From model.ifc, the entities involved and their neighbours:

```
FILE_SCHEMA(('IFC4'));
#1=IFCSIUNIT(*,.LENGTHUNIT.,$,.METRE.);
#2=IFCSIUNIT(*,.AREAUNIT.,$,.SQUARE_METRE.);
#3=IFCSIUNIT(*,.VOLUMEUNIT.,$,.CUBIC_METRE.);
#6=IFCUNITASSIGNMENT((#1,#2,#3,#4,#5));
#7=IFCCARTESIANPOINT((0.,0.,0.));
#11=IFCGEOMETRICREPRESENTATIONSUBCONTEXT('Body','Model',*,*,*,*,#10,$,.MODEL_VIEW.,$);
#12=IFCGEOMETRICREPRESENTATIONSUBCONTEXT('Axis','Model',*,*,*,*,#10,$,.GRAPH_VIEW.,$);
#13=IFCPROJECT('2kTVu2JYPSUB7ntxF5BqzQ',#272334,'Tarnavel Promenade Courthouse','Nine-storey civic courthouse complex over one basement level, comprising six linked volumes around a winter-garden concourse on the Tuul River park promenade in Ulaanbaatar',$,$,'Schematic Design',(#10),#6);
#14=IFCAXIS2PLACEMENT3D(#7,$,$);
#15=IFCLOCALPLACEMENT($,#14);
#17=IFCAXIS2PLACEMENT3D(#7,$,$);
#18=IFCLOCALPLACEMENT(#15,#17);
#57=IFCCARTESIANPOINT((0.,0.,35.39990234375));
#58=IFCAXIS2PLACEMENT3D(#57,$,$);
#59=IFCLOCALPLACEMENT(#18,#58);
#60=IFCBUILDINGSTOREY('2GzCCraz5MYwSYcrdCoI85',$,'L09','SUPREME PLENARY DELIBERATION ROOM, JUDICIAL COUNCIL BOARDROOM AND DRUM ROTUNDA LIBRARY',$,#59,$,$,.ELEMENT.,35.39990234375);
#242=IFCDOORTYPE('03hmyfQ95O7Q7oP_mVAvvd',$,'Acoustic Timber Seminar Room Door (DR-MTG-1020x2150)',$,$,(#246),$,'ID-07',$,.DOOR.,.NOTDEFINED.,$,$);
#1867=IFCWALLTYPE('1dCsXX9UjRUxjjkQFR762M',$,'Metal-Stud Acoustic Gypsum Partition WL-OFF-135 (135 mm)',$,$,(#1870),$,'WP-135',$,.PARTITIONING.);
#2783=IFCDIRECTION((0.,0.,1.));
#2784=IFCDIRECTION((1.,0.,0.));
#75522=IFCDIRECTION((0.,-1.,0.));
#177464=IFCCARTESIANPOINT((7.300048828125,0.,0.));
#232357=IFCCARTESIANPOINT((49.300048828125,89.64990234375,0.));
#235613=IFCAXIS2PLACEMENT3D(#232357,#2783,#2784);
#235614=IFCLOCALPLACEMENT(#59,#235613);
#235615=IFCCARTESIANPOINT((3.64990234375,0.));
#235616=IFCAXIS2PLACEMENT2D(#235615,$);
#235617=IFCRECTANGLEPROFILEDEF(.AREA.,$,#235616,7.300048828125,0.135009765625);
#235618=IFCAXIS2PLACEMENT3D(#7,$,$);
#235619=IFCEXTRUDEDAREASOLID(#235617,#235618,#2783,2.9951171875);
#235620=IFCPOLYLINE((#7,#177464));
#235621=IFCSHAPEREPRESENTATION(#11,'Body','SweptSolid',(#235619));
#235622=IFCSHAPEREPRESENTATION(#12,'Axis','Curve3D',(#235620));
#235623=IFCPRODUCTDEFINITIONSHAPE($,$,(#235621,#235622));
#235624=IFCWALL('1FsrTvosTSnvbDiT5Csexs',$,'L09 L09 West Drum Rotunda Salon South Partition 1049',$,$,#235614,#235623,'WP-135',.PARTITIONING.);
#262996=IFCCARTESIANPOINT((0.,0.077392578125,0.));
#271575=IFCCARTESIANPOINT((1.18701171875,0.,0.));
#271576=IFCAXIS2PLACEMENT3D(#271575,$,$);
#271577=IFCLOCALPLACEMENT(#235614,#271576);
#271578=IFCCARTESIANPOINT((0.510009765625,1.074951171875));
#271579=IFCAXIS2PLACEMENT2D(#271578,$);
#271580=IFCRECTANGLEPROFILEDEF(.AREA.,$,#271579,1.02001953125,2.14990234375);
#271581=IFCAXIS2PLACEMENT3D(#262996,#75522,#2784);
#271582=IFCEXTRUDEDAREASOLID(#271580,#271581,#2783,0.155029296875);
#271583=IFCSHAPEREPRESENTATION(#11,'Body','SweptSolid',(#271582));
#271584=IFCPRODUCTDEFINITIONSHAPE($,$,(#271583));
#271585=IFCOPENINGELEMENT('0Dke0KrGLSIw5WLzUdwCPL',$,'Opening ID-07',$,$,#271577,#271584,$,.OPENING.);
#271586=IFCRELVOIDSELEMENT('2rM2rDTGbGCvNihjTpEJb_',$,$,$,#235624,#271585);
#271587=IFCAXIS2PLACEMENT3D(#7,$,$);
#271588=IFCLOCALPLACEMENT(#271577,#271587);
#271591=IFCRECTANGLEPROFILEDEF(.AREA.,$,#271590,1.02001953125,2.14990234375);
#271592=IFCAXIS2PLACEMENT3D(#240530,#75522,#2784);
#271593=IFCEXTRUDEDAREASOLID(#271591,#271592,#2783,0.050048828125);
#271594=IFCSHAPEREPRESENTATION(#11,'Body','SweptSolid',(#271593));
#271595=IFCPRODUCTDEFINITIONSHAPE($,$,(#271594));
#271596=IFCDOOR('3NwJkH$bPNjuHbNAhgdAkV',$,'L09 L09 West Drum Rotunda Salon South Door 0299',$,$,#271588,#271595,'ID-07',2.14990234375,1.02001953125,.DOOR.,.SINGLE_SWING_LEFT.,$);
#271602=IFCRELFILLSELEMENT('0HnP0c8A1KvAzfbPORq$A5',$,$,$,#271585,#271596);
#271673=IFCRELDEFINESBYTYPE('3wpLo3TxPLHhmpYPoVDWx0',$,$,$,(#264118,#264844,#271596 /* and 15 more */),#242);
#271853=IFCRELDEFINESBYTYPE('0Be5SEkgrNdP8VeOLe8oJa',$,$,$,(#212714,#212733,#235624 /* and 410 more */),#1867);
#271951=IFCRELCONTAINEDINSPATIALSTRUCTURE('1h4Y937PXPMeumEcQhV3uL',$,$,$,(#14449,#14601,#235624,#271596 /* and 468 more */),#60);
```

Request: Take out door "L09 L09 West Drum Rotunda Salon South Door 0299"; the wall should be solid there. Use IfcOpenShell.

```python
import ifcopenshell
import ifcopenshell.api.feature
import ifcopenshell.api.root
import ifcopenshell.geom
import ifcopenshell.util.shape

model = ifcopenshell.open("model.ifc")
settings = ifcopenshell.geom.settings()


def volume(element):
    """Net volume in cubic metres, openings subtracted."""
    shape = ifcopenshell.geom.create_shape(settings, element)
    return ifcopenshell.util.shape.get_volume(shape.geometry)


door = model.by_guid("3NwJkH$bPNjuHbNAhgdAkV")
opening = door.FillsVoids[0].RelatingOpeningElement
wall = opening.VoidsElements[0].RelatingBuildingElement
before = volume(wall)

ifcopenshell.api.root.remove_product(model, product=door)
ifcopenshell.api.feature.remove_feature(model, feature=opening)

after = volume(wall)

print(f"wall volume {before:.3f} -> {after:.3f} m3")

model.write("model_edited.ifc")
```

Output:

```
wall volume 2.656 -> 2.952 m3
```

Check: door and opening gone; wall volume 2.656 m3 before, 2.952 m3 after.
